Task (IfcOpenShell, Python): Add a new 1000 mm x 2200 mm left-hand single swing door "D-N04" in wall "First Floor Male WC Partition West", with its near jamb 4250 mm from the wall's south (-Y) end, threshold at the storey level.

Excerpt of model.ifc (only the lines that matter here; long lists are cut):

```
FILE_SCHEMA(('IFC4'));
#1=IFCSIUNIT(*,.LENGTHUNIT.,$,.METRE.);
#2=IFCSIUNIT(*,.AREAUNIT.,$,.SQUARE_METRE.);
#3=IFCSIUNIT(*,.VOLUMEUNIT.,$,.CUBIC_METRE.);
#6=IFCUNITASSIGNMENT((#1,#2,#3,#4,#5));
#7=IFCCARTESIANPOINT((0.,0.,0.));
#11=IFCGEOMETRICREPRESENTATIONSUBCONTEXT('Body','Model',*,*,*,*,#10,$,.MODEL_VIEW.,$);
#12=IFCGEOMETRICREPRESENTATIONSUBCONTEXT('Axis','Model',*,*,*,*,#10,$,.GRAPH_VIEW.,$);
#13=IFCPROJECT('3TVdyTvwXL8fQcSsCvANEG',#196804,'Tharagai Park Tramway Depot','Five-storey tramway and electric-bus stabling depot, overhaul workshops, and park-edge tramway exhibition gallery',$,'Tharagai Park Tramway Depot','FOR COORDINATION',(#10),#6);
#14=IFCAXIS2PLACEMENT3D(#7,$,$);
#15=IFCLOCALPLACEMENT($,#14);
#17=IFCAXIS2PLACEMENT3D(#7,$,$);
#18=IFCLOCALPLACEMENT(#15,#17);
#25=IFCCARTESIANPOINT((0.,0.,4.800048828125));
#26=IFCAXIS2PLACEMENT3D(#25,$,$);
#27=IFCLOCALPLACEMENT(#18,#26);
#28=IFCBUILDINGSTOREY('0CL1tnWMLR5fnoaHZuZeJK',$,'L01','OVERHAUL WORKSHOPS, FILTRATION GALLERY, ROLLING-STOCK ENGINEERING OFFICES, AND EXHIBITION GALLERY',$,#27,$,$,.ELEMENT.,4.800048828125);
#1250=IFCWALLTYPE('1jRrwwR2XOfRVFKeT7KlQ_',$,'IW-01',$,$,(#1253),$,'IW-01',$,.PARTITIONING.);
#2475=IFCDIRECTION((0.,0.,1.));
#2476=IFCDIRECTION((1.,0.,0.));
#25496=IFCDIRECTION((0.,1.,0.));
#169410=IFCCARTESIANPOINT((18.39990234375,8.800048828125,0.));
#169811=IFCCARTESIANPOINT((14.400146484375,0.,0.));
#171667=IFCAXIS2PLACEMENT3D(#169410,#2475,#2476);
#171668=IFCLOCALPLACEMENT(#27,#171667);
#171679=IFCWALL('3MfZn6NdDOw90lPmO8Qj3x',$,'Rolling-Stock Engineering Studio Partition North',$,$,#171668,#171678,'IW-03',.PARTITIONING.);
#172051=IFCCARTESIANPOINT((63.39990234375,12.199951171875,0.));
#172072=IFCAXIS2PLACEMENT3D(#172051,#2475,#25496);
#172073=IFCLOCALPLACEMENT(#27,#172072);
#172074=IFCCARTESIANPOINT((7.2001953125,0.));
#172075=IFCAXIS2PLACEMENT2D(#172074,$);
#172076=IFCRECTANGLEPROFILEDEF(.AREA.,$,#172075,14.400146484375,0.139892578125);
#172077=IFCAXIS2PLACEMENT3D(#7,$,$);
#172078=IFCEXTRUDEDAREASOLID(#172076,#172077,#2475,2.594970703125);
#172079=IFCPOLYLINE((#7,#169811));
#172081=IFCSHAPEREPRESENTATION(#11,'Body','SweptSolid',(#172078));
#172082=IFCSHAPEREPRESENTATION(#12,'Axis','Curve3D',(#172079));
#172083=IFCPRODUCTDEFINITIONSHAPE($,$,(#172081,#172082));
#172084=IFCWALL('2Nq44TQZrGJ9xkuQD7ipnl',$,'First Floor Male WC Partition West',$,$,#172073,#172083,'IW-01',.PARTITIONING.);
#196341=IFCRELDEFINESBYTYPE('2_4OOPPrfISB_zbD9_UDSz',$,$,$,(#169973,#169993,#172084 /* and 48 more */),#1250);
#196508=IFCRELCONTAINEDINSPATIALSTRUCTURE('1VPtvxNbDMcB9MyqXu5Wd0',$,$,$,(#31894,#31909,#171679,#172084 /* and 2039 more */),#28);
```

```python
import numpy as np
import ifcopenshell
import ifcopenshell.api.feature
import ifcopenshell.api.geometry
import ifcopenshell.api.root
import ifcopenshell.api.spatial
import ifcopenshell.geom
import ifcopenshell.util.element
import ifcopenshell.util.placement
import ifcopenshell.util.representation
import ifcopenshell.util.shape
import ifcopenshell.util.unit

model = ifcopenshell.open("model.ifc")
unit_scale = ifcopenshell.util.unit.calculate_unit_scale(model)
settings = ifcopenshell.geom.settings()


def volume(element):
    """Net volume in cubic metres, openings subtracted."""
    shape = ifcopenshell.geom.create_shape(settings, element)
    return ifcopenshell.util.shape.get_volume(shape.geometry)


wall = model.by_id(172084)
storey = ifcopenshell.util.element.get_container(wall, ifc_class="IfcBuildingStorey")
context = ifcopenshell.util.representation.get_context(model, "Model", "Body", "MODEL_VIEW")
before = volume(wall)

width, height, from_end, sill = 1, 2.2, 4.25, 0.0  # metres

# The wall runs along its own X axis, and the end named is its -X end.
wall_shape = ifcopenshell.geom.create_shape(settings, wall)
x, y, z = ifcopenshell.util.shape.get_vertices(wall_shape.geometry).T
start = x.min() + from_end
face, thickness = float(y.min()), float(y.max() - y.min())
wall_matrix = ifcopenshell.util.placement.get_local_placement(wall.ObjectPlacement)
level = ifcopenshell.util.placement.get_local_placement(storey.ObjectPlacement)[2, 3]


def in_wall(x, y):
    """Placement at x, y metres in the wall's axes, at sill height."""
    matrix = wall_matrix.copy()
    matrix[:, 3] = wall_matrix @ np.array([x / unit_scale, y / unit_scale, 0.0, 1.0])
    matrix[2, 3] = level + sill / unit_scale
    return matrix


# Opening: a box that overshoots both wall faces by 50 mm.
opening = ifcopenshell.api.root.create_entity(model, ifc_class="IfcOpeningElement", predefined_type="OPENING")
box = ifcopenshell.api.geometry.add_wall_representation(
    model, context=context, length=width, height=height, thickness=thickness + 0.1
)
ifcopenshell.api.geometry.assign_representation(model, product=opening, representation=box)
ifcopenshell.api.geometry.edit_object_placement(model, product=opening, matrix=in_wall(start, face - 0.05), is_si=False)
ifcopenshell.api.feature.add_feature(model, feature=opening, element=wall)

door = ifcopenshell.api.root.create_entity(model, ifc_class="IfcDoor", name="D-N04", predefined_type="DOOR")
door.OverallWidth, door.OverallHeight = width / unit_scale, height / unit_scale
door.OperationType = "SINGLE_SWING_LEFT"
body = ifcopenshell.api.geometry.add_door_representation(
    model,
    context=context,
    overall_width=door.OverallWidth,
    overall_height=door.OverallHeight,
    operation_type="SINGLE_SWING_LEFT",
    lining_properties={"LiningDepth": thickness / unit_scale, "ThresholdDepth": thickness / unit_scale},
)
ifcopenshell.api.geometry.assign_representation(model, product=door, representation=body)
ifcopenshell.api.spatial.assign_container(model, products=[door], relating_structure=storey)
ifcopenshell.api.feature.add_filling(model, opening=opening, element=door)

# The lining spans the wall, so the door starts at the wall face.
ifcopenshell.api.geometry.edit_object_placement(model, product=door, matrix=in_wall(start, face), is_si=False)

after = volume(wall)

print(f"wall volume {before:.3f} -> {after:.3f} m3")

model.write("model_updated.ifc")
```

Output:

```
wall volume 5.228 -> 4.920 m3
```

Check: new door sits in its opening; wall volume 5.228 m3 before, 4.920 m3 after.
